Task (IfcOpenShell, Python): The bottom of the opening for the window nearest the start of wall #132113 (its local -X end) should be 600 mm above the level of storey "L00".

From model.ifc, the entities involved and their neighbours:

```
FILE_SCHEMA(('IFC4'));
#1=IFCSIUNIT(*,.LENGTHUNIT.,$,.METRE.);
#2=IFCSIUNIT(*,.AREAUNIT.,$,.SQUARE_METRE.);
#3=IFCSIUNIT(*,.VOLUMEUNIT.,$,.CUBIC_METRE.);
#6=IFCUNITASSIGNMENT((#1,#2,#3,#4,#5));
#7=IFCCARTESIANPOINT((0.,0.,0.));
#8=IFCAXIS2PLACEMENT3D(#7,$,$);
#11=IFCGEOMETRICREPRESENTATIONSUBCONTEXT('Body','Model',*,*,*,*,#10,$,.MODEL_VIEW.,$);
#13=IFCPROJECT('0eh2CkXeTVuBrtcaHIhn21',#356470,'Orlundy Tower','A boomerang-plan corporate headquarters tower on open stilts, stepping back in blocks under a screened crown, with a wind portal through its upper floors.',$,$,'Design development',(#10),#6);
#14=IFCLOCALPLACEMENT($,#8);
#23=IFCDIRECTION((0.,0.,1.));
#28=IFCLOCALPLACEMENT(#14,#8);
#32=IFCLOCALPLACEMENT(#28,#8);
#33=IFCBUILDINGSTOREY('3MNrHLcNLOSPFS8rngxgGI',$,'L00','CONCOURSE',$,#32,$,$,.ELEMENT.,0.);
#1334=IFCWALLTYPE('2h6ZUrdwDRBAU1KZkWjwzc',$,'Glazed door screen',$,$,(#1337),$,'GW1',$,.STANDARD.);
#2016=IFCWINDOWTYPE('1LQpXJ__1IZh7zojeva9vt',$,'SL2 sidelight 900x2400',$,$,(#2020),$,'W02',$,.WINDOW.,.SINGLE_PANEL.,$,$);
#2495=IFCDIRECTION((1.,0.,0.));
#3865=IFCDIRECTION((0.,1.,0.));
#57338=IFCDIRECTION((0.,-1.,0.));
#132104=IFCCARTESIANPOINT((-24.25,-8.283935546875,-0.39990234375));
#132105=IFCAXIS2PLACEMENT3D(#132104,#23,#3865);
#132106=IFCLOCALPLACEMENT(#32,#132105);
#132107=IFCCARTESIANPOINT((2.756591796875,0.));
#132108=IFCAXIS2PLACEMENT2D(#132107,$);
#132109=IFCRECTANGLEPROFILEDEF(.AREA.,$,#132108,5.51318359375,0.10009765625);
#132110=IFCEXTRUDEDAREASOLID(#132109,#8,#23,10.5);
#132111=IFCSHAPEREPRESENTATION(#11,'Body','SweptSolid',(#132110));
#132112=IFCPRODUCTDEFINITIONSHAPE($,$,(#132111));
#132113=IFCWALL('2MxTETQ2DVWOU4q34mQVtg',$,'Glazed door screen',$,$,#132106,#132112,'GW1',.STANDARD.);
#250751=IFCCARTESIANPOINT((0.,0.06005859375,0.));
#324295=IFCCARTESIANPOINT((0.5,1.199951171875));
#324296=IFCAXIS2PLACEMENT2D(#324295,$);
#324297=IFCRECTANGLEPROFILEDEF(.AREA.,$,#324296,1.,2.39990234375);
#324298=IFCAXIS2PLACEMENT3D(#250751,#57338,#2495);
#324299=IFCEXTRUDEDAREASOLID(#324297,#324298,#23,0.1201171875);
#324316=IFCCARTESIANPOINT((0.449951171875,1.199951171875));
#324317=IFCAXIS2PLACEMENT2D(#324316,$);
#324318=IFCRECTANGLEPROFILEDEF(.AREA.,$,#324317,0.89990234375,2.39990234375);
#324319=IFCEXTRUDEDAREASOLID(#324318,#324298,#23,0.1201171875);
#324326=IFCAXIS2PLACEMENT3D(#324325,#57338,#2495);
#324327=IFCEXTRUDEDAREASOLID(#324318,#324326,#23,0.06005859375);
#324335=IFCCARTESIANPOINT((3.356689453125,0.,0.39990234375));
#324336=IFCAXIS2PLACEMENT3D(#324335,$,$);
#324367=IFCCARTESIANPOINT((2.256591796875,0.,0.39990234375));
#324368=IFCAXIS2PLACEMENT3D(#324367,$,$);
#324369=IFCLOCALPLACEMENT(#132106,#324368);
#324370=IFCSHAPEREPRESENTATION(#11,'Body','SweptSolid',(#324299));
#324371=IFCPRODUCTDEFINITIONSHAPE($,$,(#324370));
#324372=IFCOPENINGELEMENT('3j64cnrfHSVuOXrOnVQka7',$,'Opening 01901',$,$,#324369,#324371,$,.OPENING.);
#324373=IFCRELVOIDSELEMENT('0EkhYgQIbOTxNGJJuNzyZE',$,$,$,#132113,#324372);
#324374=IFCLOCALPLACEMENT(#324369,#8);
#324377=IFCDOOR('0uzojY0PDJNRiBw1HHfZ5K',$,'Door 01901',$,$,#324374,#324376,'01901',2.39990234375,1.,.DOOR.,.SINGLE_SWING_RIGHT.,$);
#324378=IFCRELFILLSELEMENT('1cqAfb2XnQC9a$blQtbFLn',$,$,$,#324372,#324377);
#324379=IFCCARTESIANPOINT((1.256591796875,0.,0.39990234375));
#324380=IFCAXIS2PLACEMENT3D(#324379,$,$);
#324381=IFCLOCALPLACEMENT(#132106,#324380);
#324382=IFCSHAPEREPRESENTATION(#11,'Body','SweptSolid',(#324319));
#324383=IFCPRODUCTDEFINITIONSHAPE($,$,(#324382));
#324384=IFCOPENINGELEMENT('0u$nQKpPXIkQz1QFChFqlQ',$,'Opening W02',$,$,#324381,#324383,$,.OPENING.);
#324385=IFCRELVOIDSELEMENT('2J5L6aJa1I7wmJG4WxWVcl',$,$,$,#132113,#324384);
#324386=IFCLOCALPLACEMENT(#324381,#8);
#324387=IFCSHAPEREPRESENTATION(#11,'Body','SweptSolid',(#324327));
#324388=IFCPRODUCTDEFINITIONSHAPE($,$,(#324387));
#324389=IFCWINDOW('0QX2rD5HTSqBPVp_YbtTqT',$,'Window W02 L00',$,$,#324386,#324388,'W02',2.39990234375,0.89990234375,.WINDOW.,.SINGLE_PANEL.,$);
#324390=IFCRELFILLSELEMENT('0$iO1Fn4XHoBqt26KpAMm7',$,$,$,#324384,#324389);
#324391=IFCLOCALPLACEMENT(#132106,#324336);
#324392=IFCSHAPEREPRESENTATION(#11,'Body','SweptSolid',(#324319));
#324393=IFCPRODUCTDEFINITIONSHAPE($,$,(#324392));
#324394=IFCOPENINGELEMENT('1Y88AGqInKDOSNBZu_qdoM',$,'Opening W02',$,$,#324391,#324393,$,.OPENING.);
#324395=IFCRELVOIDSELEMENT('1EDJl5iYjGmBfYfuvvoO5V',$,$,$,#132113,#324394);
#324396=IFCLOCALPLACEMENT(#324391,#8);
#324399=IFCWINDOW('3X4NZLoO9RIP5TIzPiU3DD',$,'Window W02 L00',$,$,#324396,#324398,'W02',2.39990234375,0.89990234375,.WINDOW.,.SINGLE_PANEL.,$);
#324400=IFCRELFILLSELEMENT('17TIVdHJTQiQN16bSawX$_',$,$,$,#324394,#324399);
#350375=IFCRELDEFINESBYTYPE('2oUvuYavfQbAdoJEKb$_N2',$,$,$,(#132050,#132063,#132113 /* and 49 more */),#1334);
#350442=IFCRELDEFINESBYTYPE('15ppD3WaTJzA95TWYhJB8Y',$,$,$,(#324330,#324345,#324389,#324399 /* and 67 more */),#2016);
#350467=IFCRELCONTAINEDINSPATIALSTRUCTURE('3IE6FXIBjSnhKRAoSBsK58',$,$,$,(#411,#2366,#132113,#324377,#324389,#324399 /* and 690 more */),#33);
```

```python
import numpy as np
import ifcopenshell
import ifcopenshell.api.geometry
import ifcopenshell.geom
import ifcopenshell.util.element
import ifcopenshell.util.placement
import ifcopenshell.util.shape
import ifcopenshell.util.unit

model = ifcopenshell.open("model.ifc")
unit_scale = ifcopenshell.util.unit.calculate_unit_scale(model)

window = model.by_guid("0QX2rD5HTSqBPVp_YbtTqT")
opening = window.FillsVoids[0].RelatingOpeningElement
storey = ifcopenshell.util.element.get_container(window, ifc_class="IfcBuildingStorey")
level = ifcopenshell.util.placement.get_local_placement(storey.ObjectPlacement)[2, 3]

# The opening's origin need not be at the sill, so measure its lowest point.
shape = ifcopenshell.geom.create_shape(ifcopenshell.geom.settings(), opening)
bottom = ifcopenshell.util.shape.get_shape_bottom_elevation(shape, shape.geometry) / unit_scale
dz = level + 0.6 / unit_scale - bottom

shift = np.array([0.0, 0.0, dz])
# The window is placed relative to its opening, so it follows when the opening moves.
matrix = ifcopenshell.util.placement.get_local_placement(opening.ObjectPlacement)
matrix[:3, 3] += shift
ifcopenshell.api.geometry.edit_object_placement(
    model, product=opening, matrix=matrix, is_si=False, should_transform_children=True
)

print(f"moved by {dz * unit_scale:+.3f} m")

model.write("model-out.ifc")
```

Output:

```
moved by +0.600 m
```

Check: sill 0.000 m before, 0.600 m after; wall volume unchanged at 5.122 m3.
